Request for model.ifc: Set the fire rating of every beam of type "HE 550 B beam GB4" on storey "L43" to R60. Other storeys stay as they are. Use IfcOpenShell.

First a look at what the model holds.

```python
import ifcopenshell
import ifcopenshell.util.element

model = ifcopenshell.open("model.ifc")
print(model.schema)
storey = next(s for s in model.by_type("IfcBuildingStorey") if s.Name == "L43")
beams = [e for e in ifcopenshell.util.element.get_decomposition(storey) if e.is_a("IfcBeam")]
seen = {}
for e in beams:
    element_type = ifcopenshell.util.element.get_type(e)
    key = (element_type.Name if element_type != e and element_type else None, ifcopenshell.util.element.get_pset(e, "Pset_BeamCommon", "FireRating"))
    seen[key] = seen.get(key, 0) + 1
for (name, value), count in sorted(seen.items(), key=str):
    print(count, "x", name, "|", value)
```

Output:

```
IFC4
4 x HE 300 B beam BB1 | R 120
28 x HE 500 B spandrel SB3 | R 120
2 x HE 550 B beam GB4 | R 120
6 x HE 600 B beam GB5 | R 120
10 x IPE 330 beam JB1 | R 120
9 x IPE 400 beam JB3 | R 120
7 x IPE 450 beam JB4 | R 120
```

```python
import ifcopenshell
import ifcopenshell.api.pset
import ifcopenshell.util.element

model = ifcopenshell.open("model.ifc")

storey = next(s for s in model.by_type("IfcBuildingStorey") if s.Name == "L43")
beams = [e for e in ifcopenshell.util.element.get_decomposition(storey) if e.is_a("IfcBeam")]

count = 0
for e in beams:
    element_type = ifcopenshell.util.element.get_type(e)
    if element_type in (None, e) or element_type.Name != "HE 550 B beam GB4":
        continue
    found = ifcopenshell.util.element.get_pset(e, "Pset_BeamCommon", should_inherit=False)
    if found:
        pset = model.by_id(found["id"])
        if len(ifcopenshell.util.element.get_elements_by_pset(pset)) > 1:
            pset = ifcopenshell.api.pset.unshare_pset(model, products=[e], pset=pset)[0]
    else:
        pset = ifcopenshell.api.pset.add_pset(model, product=e, name="Pset_BeamCommon")
    ifcopenshell.api.pset.edit_pset(model, pset=pset, properties={"FireRating": "R60"})
    count += 1

print(count, "beams updated")

model.write("model_updated.ifc")
```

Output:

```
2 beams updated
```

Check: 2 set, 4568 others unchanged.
